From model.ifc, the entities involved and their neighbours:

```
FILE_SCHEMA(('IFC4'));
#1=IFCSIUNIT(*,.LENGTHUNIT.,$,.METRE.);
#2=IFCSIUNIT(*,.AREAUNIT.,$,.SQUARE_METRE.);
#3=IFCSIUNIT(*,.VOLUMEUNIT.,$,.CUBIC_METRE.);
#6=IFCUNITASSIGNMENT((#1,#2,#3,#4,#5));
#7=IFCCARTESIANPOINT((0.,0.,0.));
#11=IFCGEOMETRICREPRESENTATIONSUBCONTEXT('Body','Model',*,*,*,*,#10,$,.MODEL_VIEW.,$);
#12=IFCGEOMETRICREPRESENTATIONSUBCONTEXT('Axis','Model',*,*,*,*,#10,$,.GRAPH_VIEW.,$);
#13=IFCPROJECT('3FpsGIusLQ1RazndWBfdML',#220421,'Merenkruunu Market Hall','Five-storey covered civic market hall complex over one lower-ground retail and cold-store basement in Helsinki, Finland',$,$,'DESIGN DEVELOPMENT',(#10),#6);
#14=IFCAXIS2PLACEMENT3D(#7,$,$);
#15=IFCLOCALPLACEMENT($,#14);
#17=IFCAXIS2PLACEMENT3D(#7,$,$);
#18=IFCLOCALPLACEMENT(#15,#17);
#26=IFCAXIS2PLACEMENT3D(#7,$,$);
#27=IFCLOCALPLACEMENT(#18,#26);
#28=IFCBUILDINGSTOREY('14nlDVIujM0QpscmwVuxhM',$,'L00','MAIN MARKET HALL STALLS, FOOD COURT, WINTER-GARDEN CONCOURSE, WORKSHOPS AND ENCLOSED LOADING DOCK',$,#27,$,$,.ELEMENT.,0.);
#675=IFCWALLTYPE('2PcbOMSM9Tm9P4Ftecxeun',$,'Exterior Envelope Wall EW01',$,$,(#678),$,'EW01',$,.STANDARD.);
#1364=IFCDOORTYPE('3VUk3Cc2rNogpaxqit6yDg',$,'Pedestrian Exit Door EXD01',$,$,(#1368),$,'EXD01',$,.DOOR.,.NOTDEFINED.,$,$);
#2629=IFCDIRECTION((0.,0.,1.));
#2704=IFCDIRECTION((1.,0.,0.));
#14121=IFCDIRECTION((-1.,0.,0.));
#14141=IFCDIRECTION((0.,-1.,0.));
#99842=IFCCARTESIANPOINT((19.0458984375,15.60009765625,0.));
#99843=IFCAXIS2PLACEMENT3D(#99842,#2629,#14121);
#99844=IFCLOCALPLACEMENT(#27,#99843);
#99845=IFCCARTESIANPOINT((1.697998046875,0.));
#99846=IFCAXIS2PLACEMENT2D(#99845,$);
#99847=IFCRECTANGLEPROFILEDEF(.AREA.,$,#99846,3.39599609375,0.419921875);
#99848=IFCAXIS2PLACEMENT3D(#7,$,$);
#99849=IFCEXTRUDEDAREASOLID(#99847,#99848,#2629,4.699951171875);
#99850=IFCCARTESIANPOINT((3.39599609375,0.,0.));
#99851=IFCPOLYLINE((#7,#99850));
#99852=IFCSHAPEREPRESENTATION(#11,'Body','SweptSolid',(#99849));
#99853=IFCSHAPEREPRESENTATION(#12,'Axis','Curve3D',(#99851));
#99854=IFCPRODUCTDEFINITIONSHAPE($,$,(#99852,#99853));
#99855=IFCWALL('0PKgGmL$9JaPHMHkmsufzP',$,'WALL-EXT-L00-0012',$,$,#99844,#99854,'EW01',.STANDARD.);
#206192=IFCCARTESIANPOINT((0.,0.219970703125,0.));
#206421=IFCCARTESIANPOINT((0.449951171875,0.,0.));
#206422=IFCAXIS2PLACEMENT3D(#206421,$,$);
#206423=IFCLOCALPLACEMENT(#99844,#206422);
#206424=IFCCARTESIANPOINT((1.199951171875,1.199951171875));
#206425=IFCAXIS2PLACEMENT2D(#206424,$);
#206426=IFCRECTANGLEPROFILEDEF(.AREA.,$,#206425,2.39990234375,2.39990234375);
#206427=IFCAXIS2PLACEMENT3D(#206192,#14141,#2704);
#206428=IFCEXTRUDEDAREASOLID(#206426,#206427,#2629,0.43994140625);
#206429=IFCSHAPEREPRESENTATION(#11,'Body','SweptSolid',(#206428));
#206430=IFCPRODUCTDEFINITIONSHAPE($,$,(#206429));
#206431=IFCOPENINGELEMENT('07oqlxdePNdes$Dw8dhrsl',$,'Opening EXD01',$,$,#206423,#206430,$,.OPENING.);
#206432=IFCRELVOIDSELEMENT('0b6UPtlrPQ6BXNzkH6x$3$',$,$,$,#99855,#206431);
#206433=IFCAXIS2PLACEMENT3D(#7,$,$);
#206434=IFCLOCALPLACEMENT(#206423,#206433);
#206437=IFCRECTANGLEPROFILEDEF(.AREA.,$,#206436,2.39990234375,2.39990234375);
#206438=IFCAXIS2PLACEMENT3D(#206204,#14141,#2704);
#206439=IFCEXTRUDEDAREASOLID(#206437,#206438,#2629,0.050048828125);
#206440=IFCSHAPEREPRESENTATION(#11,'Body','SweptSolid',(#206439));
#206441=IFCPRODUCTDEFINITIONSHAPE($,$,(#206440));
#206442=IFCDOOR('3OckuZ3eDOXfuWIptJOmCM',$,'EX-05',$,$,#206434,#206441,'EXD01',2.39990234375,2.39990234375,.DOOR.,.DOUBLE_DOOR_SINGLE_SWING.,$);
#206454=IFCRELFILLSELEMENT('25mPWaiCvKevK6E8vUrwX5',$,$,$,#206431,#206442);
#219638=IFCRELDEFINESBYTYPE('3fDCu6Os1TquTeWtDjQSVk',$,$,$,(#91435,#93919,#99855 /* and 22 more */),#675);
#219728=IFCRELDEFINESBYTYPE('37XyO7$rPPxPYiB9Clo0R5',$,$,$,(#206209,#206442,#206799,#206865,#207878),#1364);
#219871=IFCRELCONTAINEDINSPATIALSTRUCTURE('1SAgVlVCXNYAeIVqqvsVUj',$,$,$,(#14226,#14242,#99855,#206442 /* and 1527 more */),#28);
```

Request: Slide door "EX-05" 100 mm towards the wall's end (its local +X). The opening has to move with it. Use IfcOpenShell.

```python
import ifcopenshell
import ifcopenshell.api.geometry
import ifcopenshell.util.placement

model = ifcopenshell.open("model.ifc")

door = model.by_guid("3OckuZ3eDOXfuWIptJOmCM")
opening = door.FillsVoids[0].RelatingOpeningElement
wall = opening.VoidsElements[0].RelatingBuildingElement

wall_matrix = ifcopenshell.util.placement.get_local_placement(wall.ObjectPlacement)
shift = wall_matrix[:3, 0] * 0.1
before = ifcopenshell.util.placement.get_local_placement(door.ObjectPlacement)[:3, 3].copy()

# The door is placed relative to its opening, so it follows when the opening moves.
matrix = ifcopenshell.util.placement.get_local_placement(opening.ObjectPlacement)
matrix[:3, 3] += shift
ifcopenshell.api.geometry.edit_object_placement(
    model, product=opening, matrix=matrix, is_si=False, should_transform_children=True
)

after = ifcopenshell.util.placement.get_local_placement(door.ObjectPlacement)[:3, 3]
print("door moved by", (after - before).round(3) + 0.0)

model.write("model-out.ifc")
```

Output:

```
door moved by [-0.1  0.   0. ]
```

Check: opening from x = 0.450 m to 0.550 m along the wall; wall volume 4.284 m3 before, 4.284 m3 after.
